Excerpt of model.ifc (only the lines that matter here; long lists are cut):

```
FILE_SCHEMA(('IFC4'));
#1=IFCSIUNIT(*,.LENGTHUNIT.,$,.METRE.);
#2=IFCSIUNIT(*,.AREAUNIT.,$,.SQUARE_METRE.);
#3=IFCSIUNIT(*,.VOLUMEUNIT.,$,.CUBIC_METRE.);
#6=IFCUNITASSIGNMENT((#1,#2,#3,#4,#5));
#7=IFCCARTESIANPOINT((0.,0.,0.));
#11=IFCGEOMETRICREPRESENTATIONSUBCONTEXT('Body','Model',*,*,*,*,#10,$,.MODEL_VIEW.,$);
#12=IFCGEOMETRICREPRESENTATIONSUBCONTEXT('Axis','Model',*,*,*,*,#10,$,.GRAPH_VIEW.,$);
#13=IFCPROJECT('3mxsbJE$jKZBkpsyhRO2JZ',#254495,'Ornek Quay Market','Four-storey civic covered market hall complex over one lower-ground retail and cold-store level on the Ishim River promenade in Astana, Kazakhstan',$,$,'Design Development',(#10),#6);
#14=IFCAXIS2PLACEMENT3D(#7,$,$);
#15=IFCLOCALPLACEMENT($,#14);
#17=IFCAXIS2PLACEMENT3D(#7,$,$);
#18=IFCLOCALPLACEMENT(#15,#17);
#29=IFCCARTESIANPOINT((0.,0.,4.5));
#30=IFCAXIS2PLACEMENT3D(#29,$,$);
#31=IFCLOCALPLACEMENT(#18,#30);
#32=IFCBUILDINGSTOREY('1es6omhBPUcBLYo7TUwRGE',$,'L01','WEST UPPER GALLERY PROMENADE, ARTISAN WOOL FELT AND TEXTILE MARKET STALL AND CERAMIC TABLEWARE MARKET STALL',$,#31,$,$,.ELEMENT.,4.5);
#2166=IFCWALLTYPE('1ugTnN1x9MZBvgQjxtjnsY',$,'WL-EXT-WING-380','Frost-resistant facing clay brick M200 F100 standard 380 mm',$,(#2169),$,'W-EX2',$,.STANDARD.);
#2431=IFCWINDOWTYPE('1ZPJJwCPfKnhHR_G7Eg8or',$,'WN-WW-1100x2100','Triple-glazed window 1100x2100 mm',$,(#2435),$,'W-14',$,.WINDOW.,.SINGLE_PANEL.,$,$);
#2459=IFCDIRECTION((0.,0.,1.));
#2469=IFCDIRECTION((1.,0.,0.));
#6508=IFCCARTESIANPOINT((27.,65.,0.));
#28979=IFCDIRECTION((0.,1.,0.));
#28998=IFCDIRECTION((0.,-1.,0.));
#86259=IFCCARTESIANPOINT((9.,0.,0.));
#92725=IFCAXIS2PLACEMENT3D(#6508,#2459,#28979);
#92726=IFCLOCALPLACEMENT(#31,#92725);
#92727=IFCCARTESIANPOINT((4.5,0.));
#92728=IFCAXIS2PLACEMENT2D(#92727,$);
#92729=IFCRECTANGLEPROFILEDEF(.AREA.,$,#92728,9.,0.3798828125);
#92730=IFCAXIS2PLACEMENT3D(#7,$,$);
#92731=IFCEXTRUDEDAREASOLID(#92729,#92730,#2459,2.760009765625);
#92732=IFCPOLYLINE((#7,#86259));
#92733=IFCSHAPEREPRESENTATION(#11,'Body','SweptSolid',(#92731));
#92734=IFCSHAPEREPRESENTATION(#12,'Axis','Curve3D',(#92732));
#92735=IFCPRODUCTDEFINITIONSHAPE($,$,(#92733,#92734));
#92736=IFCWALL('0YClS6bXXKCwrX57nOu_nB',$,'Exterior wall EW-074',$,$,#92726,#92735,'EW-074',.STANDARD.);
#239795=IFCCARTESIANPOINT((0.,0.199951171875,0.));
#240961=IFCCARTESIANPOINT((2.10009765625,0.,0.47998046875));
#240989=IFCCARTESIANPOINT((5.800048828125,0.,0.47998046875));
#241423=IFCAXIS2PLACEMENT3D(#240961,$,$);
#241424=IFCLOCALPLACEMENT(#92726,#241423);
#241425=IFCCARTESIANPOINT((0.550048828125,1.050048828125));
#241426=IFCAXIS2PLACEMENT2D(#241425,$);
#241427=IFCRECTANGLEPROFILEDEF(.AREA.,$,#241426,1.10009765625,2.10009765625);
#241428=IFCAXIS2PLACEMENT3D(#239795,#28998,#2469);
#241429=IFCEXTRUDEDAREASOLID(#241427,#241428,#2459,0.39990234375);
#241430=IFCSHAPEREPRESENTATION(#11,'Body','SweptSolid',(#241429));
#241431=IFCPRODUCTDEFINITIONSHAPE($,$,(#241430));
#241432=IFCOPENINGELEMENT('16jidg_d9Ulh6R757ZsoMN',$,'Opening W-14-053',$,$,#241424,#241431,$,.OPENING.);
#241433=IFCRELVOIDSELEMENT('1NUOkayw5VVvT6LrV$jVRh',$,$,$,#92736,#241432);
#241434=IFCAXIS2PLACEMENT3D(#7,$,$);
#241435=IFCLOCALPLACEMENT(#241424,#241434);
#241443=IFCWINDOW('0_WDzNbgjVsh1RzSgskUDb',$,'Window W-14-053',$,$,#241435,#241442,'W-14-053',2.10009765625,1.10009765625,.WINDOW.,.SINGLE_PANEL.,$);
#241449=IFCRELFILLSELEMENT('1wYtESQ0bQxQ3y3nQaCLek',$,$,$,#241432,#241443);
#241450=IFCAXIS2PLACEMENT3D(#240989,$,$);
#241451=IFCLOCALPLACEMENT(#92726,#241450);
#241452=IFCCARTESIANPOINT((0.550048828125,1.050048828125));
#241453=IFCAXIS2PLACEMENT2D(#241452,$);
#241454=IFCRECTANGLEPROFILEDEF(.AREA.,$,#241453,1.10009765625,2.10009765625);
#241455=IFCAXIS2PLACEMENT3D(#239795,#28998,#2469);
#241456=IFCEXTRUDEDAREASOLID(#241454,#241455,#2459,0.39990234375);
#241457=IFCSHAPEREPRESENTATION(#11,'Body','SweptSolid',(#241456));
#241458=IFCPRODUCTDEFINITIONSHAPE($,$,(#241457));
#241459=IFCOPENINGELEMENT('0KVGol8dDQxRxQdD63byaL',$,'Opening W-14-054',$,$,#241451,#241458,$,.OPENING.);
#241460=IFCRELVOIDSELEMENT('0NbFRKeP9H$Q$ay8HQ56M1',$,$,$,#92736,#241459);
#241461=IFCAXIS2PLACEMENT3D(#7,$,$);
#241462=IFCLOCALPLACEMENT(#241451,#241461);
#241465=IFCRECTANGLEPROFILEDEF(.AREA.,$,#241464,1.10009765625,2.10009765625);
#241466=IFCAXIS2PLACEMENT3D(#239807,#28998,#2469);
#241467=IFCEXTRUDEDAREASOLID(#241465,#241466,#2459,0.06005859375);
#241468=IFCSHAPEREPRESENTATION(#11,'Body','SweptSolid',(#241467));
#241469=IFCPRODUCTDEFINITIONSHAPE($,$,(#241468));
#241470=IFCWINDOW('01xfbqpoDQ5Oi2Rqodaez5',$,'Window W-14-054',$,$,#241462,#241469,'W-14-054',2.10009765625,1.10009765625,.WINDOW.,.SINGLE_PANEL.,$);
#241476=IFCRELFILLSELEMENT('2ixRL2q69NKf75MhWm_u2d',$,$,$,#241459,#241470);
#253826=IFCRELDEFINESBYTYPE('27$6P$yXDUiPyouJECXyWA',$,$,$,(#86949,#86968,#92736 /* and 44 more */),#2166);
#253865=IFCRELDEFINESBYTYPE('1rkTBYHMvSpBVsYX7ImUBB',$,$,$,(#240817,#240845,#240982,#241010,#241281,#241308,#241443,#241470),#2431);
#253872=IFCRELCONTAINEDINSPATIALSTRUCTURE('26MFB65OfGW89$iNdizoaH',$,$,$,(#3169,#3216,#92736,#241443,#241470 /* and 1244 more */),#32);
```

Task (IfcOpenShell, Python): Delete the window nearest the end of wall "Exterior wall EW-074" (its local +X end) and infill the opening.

```python
import ifcopenshell
import ifcopenshell.api.feature
import ifcopenshell.api.root
import ifcopenshell.geom
import ifcopenshell.util.shape

model = ifcopenshell.open("model.ifc")
settings = ifcopenshell.geom.settings()


def volume(element):
    """Net volume in cubic metres, openings subtracted."""
    shape = ifcopenshell.geom.create_shape(settings, element)
    return ifcopenshell.util.shape.get_volume(shape.geometry)


window = model.by_id(241470)
opening = window.FillsVoids[0].RelatingOpeningElement
wall = opening.VoidsElements[0].RelatingBuildingElement
before = volume(wall)

ifcopenshell.api.root.remove_product(model, product=window)
ifcopenshell.api.feature.remove_feature(model, feature=opening)

after = volume(wall)

print(f"wall volume {before:.3f} -> {after:.3f} m3")

model.write("model_rev.ifc")
```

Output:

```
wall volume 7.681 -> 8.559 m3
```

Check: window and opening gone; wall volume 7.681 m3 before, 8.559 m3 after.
